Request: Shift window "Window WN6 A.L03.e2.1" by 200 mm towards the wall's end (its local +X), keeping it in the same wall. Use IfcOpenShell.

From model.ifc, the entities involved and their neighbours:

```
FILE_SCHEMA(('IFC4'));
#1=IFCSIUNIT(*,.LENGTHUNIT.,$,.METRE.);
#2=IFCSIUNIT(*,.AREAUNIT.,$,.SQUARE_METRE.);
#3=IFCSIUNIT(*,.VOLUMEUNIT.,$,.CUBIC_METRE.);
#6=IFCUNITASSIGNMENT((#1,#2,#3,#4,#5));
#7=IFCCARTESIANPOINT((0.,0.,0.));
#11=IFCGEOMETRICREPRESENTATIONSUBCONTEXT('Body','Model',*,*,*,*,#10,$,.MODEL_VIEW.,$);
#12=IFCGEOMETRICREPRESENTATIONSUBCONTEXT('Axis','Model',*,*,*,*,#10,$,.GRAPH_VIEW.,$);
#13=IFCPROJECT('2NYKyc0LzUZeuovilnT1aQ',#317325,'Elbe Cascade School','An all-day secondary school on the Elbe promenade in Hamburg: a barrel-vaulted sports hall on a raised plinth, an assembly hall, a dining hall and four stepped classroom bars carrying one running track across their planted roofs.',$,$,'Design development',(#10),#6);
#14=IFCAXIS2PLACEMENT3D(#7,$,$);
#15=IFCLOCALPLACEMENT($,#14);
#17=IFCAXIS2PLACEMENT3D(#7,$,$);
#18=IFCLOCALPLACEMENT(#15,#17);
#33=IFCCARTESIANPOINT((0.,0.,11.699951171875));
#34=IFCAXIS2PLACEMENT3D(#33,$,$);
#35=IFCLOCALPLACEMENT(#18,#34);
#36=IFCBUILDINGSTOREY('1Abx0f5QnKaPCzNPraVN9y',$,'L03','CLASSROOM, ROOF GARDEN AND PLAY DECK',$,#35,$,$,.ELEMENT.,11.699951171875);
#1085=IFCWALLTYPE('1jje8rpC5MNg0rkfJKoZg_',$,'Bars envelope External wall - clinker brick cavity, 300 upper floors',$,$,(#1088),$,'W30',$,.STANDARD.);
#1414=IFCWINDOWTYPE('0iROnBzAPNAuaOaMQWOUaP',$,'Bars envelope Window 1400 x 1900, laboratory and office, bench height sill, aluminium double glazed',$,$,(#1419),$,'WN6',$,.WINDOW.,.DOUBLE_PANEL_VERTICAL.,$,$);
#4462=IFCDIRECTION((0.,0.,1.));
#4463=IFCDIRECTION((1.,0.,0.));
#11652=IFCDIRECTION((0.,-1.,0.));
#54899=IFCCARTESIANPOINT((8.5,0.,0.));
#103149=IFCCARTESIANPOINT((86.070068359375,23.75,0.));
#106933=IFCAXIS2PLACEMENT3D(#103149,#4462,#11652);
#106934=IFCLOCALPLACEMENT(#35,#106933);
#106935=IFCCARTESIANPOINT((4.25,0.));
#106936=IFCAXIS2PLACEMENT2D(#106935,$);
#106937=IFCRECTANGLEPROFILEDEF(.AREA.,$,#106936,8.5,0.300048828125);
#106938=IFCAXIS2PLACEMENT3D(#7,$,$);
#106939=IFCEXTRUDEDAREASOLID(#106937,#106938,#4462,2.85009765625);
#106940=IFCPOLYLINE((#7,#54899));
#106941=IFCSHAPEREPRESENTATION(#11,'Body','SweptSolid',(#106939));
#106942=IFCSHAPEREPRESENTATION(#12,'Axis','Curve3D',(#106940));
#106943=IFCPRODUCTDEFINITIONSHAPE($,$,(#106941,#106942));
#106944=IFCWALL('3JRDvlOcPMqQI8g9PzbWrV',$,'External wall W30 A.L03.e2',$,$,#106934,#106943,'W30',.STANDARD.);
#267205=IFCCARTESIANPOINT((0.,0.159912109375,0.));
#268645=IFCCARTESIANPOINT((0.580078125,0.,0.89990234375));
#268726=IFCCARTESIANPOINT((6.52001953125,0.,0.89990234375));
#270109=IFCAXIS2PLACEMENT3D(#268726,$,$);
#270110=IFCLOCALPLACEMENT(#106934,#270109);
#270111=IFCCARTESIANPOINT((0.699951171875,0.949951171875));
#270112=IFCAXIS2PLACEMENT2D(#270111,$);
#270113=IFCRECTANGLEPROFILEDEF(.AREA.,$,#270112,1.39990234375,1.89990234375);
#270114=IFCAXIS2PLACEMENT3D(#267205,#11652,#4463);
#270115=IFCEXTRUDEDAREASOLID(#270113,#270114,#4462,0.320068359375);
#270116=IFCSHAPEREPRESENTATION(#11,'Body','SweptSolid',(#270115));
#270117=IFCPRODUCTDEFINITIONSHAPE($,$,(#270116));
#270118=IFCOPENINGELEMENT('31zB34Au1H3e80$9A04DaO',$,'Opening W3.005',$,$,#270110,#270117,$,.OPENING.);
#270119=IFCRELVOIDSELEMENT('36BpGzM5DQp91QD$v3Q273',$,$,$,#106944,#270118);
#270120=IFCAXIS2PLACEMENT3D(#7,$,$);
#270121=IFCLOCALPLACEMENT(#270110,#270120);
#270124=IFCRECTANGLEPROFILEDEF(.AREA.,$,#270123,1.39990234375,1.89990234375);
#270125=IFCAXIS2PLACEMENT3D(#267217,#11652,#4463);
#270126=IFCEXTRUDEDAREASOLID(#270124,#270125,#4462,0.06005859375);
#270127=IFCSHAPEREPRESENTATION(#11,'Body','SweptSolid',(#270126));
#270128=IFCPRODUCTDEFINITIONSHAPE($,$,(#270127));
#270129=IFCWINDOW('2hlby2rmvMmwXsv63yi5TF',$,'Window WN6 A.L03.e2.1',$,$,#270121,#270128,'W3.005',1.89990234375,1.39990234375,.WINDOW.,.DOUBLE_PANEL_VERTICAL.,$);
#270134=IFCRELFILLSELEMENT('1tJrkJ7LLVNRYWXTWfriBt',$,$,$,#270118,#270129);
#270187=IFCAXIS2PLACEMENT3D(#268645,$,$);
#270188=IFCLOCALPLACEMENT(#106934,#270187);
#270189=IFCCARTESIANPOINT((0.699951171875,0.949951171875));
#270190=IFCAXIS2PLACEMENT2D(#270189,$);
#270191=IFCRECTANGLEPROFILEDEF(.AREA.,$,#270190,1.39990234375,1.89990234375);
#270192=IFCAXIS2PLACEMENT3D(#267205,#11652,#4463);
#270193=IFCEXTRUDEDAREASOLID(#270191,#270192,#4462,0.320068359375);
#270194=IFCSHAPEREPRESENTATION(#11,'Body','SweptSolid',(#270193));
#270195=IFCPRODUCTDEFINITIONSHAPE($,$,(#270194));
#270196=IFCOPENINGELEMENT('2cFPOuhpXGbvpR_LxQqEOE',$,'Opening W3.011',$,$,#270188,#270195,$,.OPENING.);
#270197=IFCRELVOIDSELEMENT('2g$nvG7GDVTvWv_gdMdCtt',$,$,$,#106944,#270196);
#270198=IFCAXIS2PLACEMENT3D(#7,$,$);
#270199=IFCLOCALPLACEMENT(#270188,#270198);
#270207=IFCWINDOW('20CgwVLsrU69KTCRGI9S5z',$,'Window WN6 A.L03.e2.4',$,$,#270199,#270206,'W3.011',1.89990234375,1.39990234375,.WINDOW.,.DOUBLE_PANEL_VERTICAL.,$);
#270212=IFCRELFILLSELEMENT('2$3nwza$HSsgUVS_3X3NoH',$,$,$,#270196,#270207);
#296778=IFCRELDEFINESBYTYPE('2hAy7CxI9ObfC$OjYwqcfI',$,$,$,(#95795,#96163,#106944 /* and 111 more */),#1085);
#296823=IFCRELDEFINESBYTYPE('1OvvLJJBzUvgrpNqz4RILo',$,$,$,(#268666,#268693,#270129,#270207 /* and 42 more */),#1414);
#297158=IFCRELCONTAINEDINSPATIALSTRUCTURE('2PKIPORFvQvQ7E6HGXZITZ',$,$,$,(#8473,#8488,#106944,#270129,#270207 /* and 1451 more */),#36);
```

```python
import ifcopenshell
import ifcopenshell.api.geometry
import ifcopenshell.util.placement
import ifcopenshell.util.unit

model = ifcopenshell.open("model.ifc")
unit_scale = ifcopenshell.util.unit.calculate_unit_scale(model)

window = model.by_guid("2hlby2rmvMmwXsv63yi5TF")
opening = window.FillsVoids[0].RelatingOpeningElement
wall = opening.VoidsElements[0].RelatingBuildingElement

wall_matrix = ifcopenshell.util.placement.get_local_placement(wall.ObjectPlacement)
shift = wall_matrix[:3, 0] * 0.2 / unit_scale
before = ifcopenshell.util.placement.get_local_placement(window.ObjectPlacement)[:3, 3].copy()

# The window is placed relative to its opening, so it follows when the opening moves.
matrix = ifcopenshell.util.placement.get_local_placement(opening.ObjectPlacement)
matrix[:3, 3] += shift
ifcopenshell.api.geometry.edit_object_placement(
    model, product=opening, matrix=matrix, is_si=False, should_transform_children=True
)

after = ifcopenshell.util.placement.get_local_placement(window.ObjectPlacement)[:3, 3]
print("window moved by", (after - before).round(3) + 0.0)

model.write("model-out.ifc")
```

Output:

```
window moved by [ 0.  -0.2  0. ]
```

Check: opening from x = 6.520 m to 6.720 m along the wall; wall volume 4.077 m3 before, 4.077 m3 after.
